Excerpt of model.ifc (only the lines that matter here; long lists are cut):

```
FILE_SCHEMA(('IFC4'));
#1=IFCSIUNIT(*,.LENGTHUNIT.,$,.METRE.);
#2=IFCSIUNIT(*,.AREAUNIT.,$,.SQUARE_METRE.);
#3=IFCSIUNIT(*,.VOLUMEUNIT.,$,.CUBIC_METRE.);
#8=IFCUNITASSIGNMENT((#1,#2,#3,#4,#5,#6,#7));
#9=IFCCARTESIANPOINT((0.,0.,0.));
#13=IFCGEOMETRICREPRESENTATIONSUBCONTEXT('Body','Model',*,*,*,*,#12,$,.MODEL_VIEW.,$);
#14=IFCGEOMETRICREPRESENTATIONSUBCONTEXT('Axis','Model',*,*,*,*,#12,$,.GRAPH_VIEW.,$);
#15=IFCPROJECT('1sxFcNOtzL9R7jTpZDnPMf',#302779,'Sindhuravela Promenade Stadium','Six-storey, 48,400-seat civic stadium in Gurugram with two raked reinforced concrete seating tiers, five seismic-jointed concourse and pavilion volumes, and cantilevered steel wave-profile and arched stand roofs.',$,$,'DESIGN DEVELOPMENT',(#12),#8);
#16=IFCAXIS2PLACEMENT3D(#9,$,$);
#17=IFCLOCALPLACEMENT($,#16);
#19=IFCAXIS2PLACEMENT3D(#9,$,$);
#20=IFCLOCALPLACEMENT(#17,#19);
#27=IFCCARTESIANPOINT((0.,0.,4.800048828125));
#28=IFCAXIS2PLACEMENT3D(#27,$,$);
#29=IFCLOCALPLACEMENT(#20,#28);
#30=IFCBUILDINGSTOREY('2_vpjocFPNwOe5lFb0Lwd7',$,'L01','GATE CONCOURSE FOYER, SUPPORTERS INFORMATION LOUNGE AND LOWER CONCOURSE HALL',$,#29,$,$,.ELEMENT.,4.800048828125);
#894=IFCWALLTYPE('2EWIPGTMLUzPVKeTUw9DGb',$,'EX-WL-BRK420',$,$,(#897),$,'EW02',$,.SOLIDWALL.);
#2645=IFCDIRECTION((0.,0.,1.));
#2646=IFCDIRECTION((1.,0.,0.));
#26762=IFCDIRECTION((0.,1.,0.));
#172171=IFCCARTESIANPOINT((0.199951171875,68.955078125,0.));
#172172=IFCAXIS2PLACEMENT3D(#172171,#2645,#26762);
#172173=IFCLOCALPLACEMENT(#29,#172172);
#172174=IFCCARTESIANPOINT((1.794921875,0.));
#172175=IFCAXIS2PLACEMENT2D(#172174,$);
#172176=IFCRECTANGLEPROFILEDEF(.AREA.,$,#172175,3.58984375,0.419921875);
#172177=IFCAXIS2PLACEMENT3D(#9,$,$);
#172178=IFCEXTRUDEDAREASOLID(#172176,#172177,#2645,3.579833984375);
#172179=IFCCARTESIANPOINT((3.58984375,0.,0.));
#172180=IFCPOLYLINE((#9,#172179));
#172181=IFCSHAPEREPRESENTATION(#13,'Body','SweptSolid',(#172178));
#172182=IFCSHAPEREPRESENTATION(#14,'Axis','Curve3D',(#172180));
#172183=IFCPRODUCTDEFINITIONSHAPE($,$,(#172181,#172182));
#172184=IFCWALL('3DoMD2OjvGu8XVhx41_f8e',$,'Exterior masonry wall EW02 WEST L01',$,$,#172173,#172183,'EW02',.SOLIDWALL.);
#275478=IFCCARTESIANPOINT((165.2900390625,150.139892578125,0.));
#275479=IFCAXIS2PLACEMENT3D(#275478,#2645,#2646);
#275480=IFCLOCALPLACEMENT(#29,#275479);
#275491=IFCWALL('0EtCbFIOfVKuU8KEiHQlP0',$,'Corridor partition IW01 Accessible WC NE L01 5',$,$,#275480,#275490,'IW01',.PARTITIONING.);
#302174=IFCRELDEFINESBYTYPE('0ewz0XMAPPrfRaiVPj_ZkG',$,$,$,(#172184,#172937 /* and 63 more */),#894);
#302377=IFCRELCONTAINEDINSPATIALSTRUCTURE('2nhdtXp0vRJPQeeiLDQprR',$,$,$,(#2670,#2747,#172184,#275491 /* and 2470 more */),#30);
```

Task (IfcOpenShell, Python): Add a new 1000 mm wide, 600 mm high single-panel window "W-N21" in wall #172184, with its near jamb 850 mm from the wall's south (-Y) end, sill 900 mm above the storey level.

```python
import numpy as np
import ifcopenshell
import ifcopenshell.api.feature
import ifcopenshell.api.geometry
import ifcopenshell.api.root
import ifcopenshell.api.spatial
import ifcopenshell.geom
import ifcopenshell.util.element
import ifcopenshell.util.placement
import ifcopenshell.util.representation
import ifcopenshell.util.shape
import ifcopenshell.util.unit

model = ifcopenshell.open("model.ifc")
unit_scale = ifcopenshell.util.unit.calculate_unit_scale(model)
settings = ifcopenshell.geom.settings()


def volume(element):
    """Net volume in cubic metres, openings subtracted."""
    shape = ifcopenshell.geom.create_shape(settings, element)
    return ifcopenshell.util.shape.get_volume(shape.geometry)


wall = model.by_id(172184)
storey = ifcopenshell.util.element.get_container(wall, ifc_class="IfcBuildingStorey")
context = ifcopenshell.util.representation.get_context(model, "Model", "Body", "MODEL_VIEW")
before = volume(wall)

width, height, from_end, sill = 1, 0.6, 0.85, 0.9  # metres

# The wall runs along its own X axis, and the end named is its -X end.
wall_shape = ifcopenshell.geom.create_shape(settings, wall)
x, y, z = ifcopenshell.util.shape.get_vertices(wall_shape.geometry).T
start = x.min() + from_end
face, thickness = float(y.min()), float(y.max() - y.min())
wall_matrix = ifcopenshell.util.placement.get_local_placement(wall.ObjectPlacement)
level = ifcopenshell.util.placement.get_local_placement(storey.ObjectPlacement)[2, 3]


def in_wall(x, y):
    """Placement at x, y metres in the wall's axes, at sill height."""
    matrix = wall_matrix.copy()
    matrix[:, 3] = wall_matrix @ np.array([x / unit_scale, y / unit_scale, 0.0, 1.0])
    matrix[2, 3] = level + sill / unit_scale
    return matrix


# Opening: a box that overshoots both wall faces by 50 mm.
opening = ifcopenshell.api.root.create_entity(model, ifc_class="IfcOpeningElement", predefined_type="OPENING")
box = ifcopenshell.api.geometry.add_wall_representation(
    model, context=context, length=width, height=height, thickness=thickness + 0.1
)
ifcopenshell.api.geometry.assign_representation(model, product=opening, representation=box)
ifcopenshell.api.geometry.edit_object_placement(model, product=opening, matrix=in_wall(start, face - 0.05), is_si=False)
ifcopenshell.api.feature.add_feature(model, feature=opening, element=wall)

window = ifcopenshell.api.root.create_entity(model, ifc_class="IfcWindow", name="W-N21", predefined_type="WINDOW")
window.OverallWidth, window.OverallHeight = width / unit_scale, height / unit_scale
window.PartitioningType = "SINGLE_PANEL"
body = ifcopenshell.api.geometry.add_window_representation(
    model,
    context=context,
    overall_width=window.OverallWidth,
    overall_height=window.OverallHeight,
    partition_type="SINGLE_PANEL",
)
ifcopenshell.api.geometry.assign_representation(model, product=window, representation=body)
ifcopenshell.api.spatial.assign_container(model, products=[window], relating_structure=storey)
ifcopenshell.api.feature.add_filling(model, opening=opening, element=window)

# Centre the window in the wall's thickness.
ifcopenshell.api.geometry.edit_object_placement(model, product=window, matrix=in_wall(start, face), is_si=False)
window_shape = ifcopenshell.geom.create_shape(settings, window)
depth = ifcopenshell.util.shape.get_vertices(window_shape.geometry)[:, 1]
offset = face + thickness / 2 - (depth.min() + depth.max()) / 2
ifcopenshell.api.geometry.edit_object_placement(model, product=window, matrix=in_wall(start, offset), is_si=False)

after = volume(wall)

print(f"wall volume {before:.3f} -> {after:.3f} m3")

model.write("model_updated.ifc")
```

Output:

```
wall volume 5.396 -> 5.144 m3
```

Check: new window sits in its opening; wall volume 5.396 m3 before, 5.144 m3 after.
